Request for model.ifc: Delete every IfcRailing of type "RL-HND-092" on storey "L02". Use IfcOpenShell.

First a look at what the model holds.

```python
import ifcopenshell
import ifcopenshell.util.element

model = ifcopenshell.open("model.ifc")
print(model.schema)
storey = next(s for s in model.by_type("IfcBuildingStorey") if s.Name == "L02")
railings = [e for e in ifcopenshell.util.element.get_decomposition(storey) if e.is_a("IfcRailing")]
seen = {}
for e in railings:
    element_type = ifcopenshell.util.element.get_type(e)
    name = element_type.Name if element_type not in (None, e) else None
    seen[name] = seen.get(name, 0) + 1
for name, count in sorted(seen.items(), key=str):
    print(count, "x", name)
```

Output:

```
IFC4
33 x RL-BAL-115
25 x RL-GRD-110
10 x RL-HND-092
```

```python
import ifcopenshell
import ifcopenshell.api.root
import ifcopenshell.util.element

model = ifcopenshell.open("model.ifc")

storey = next(s for s in model.by_type("IfcBuildingStorey") if s.Name == "L02")
railings = [e for e in ifcopenshell.util.element.get_decomposition(storey) if e.is_a("IfcRailing")]
targets = [e for e in railings if (t := ifcopenshell.util.element.get_type(e)) not in (None, e) and t.Name == "RL-HND-092"]

for e in targets:
    ifcopenshell.api.root.remove_product(model, product=e)
print(len(targets), "removed")

model.write("model-out.ifc")
```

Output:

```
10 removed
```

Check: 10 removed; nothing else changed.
